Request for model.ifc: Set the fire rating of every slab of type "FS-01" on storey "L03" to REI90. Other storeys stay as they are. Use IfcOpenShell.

First a look at what the model holds.

```python
import ifcopenshell
import ifcopenshell.util.element

model = ifcopenshell.open("model.ifc")
print(model.schema)
storey = next(s for s in model.by_type("IfcBuildingStorey") if s.Name == "L03")
slabs = [e for e in ifcopenshell.util.element.get_decomposition(storey) if e.is_a("IfcSlab")]
seen = {}
for e in slabs:
    element_type = ifcopenshell.util.element.get_type(e)
    key = (element_type.Name if element_type != e and element_type else None, ifcopenshell.util.element.get_pset(e, "Pset_SlabCommon", "FireRating"))
    seen[key] = seen.get(key, 0) + 1
for (name, value), count in sorted(seen.items(), key=str):
    print(count, "x", name, "|", value)
```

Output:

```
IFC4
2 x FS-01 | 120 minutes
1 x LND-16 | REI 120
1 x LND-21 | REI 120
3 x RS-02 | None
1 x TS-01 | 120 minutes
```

```python
import ifcopenshell
import ifcopenshell.api.pset
import ifcopenshell.util.element

model = ifcopenshell.open("model.ifc")

storey = next(s for s in model.by_type("IfcBuildingStorey") if s.Name == "L03")
slabs = [e for e in ifcopenshell.util.element.get_decomposition(storey) if e.is_a("IfcSlab")]

count = 0
for e in slabs:
    element_type = ifcopenshell.util.element.get_type(e)
    if element_type in (None, e) or element_type.Name != "FS-01":
        continue
    # add_pset returns the element's existing set when there is one.
    pset = ifcopenshell.api.pset.add_pset(model, product=e, name="Pset_SlabCommon")
    ifcopenshell.api.pset.edit_pset(model, pset=pset, properties={"FireRating": "REI90"})
    count += 1

print(count, "slabs updated")

model.write("model_v2.ifc")
```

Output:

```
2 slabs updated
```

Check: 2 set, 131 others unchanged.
